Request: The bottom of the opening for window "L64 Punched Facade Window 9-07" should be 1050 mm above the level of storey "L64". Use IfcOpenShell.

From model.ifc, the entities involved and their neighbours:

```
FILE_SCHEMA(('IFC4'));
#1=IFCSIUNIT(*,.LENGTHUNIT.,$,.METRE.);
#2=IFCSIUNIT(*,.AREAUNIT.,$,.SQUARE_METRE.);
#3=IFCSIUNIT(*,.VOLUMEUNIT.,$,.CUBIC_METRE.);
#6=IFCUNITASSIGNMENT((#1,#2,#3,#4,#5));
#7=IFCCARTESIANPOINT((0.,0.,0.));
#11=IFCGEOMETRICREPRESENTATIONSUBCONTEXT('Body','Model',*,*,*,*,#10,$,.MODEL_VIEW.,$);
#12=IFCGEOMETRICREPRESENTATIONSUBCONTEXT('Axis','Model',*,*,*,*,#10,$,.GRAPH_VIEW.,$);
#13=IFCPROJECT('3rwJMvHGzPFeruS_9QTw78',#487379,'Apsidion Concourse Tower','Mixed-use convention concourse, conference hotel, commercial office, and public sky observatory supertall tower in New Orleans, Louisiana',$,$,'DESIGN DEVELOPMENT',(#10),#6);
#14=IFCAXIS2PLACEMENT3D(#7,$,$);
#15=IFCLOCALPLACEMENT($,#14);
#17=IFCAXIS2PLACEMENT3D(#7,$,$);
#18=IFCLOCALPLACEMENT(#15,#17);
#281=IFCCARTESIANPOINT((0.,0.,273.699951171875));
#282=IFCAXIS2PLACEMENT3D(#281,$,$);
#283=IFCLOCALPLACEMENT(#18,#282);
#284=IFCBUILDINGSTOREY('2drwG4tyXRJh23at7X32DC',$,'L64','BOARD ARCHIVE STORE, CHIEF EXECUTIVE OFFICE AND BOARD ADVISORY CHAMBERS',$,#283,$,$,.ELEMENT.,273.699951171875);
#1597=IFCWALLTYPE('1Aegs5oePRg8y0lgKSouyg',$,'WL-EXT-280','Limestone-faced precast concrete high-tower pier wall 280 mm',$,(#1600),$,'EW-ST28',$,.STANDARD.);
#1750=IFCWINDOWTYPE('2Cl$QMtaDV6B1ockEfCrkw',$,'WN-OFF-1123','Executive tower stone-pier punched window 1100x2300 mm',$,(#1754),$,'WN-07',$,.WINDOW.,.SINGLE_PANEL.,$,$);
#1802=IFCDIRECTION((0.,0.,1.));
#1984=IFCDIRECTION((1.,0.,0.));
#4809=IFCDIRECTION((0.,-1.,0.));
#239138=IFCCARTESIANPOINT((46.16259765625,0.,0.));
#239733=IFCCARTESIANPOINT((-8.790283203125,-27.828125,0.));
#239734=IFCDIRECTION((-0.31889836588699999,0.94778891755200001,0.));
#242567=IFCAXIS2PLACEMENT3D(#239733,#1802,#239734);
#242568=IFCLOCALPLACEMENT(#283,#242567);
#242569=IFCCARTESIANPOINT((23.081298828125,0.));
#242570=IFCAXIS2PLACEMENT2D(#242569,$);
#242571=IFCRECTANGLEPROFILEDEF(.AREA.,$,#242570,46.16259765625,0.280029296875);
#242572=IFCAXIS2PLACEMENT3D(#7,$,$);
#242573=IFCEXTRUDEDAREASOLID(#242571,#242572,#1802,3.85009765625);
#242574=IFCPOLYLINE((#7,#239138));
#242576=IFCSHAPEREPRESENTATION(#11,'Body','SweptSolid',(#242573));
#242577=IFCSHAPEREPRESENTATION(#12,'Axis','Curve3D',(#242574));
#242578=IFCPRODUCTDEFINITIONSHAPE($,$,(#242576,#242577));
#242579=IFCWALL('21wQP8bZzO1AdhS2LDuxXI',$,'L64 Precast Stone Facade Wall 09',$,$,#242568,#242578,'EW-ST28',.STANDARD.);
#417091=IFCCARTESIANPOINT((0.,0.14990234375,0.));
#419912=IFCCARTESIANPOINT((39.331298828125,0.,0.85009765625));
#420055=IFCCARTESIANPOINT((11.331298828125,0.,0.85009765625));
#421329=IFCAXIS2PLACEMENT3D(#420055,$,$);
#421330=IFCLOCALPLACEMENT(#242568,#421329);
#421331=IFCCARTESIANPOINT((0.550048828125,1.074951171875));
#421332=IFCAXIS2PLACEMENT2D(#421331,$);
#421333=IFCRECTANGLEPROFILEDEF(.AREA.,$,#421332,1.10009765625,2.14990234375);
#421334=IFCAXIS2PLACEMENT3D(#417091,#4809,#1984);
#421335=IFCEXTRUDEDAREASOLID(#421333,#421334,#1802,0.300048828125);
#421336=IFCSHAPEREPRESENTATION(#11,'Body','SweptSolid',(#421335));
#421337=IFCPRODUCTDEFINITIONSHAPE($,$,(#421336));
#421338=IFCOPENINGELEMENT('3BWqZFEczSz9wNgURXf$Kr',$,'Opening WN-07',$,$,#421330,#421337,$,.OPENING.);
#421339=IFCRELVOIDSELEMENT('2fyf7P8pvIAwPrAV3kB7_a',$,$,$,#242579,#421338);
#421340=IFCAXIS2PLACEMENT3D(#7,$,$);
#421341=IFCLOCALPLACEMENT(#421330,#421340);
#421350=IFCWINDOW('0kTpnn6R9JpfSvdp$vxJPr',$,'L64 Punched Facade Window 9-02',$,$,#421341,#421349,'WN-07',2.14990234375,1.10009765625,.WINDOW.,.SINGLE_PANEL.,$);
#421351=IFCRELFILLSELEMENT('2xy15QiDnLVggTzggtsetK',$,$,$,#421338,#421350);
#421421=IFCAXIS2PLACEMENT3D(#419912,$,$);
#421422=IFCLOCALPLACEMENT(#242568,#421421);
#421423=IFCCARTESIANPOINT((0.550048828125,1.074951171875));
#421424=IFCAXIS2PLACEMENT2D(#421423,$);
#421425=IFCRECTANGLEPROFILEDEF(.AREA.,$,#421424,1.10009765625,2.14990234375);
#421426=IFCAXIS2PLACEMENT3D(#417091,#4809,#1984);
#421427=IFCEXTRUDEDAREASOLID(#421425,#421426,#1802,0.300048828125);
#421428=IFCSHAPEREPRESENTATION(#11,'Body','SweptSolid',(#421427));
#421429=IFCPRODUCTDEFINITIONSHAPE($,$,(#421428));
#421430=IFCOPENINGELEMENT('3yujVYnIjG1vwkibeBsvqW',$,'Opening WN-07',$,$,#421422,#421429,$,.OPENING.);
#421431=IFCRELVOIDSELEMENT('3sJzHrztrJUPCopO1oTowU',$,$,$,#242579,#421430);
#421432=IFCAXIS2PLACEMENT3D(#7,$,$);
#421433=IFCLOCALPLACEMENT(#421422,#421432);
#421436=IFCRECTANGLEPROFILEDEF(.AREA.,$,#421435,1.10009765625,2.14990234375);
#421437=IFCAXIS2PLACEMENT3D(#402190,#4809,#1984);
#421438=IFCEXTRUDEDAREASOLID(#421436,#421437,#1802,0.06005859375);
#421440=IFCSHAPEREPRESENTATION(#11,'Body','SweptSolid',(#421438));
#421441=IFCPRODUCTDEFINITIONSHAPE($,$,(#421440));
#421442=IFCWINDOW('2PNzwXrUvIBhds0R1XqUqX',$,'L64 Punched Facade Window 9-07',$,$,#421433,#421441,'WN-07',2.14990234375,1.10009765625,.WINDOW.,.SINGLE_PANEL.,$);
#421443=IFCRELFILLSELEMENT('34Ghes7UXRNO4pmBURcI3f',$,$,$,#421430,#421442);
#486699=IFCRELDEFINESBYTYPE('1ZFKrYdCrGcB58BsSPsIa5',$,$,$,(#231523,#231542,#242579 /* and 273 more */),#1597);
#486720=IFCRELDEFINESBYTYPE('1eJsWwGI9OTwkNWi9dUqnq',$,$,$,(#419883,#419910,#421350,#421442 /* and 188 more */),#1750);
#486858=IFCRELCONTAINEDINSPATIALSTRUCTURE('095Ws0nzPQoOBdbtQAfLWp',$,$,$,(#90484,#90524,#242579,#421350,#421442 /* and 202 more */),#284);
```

```python
import numpy as np
import ifcopenshell
import ifcopenshell.api.geometry
import ifcopenshell.geom
import ifcopenshell.util.element
import ifcopenshell.util.placement
import ifcopenshell.util.shape
import ifcopenshell.util.unit

model = ifcopenshell.open("model.ifc")
unit_scale = ifcopenshell.util.unit.calculate_unit_scale(model)

window = model.by_guid("2PNzwXrUvIBhds0R1XqUqX")
opening = window.FillsVoids[0].RelatingOpeningElement
storey = ifcopenshell.util.element.get_container(window, ifc_class="IfcBuildingStorey")
level = ifcopenshell.util.placement.get_local_placement(storey.ObjectPlacement)[2, 3]

# The opening's origin need not be at the sill, so measure its lowest point.
shape = ifcopenshell.geom.create_shape(ifcopenshell.geom.settings(), opening)
bottom = ifcopenshell.util.shape.get_shape_bottom_elevation(shape, shape.geometry) / unit_scale
dz = level + 1.05 - bottom

shift = np.array([0.0, 0.0, dz])
# The window is placed relative to its opening, so it follows when the opening moves.
matrix = ifcopenshell.util.placement.get_local_placement(opening.ObjectPlacement)
matrix[:3, 3] += shift
ifcopenshell.api.geometry.edit_object_placement(
    model, product=opening, matrix=matrix, is_si=False, should_transform_children=True
)

print(f"moved by {dz * unit_scale:+.3f} m")

model.write("model_updated.ifc")
```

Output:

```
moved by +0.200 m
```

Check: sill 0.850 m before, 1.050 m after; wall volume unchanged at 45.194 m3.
